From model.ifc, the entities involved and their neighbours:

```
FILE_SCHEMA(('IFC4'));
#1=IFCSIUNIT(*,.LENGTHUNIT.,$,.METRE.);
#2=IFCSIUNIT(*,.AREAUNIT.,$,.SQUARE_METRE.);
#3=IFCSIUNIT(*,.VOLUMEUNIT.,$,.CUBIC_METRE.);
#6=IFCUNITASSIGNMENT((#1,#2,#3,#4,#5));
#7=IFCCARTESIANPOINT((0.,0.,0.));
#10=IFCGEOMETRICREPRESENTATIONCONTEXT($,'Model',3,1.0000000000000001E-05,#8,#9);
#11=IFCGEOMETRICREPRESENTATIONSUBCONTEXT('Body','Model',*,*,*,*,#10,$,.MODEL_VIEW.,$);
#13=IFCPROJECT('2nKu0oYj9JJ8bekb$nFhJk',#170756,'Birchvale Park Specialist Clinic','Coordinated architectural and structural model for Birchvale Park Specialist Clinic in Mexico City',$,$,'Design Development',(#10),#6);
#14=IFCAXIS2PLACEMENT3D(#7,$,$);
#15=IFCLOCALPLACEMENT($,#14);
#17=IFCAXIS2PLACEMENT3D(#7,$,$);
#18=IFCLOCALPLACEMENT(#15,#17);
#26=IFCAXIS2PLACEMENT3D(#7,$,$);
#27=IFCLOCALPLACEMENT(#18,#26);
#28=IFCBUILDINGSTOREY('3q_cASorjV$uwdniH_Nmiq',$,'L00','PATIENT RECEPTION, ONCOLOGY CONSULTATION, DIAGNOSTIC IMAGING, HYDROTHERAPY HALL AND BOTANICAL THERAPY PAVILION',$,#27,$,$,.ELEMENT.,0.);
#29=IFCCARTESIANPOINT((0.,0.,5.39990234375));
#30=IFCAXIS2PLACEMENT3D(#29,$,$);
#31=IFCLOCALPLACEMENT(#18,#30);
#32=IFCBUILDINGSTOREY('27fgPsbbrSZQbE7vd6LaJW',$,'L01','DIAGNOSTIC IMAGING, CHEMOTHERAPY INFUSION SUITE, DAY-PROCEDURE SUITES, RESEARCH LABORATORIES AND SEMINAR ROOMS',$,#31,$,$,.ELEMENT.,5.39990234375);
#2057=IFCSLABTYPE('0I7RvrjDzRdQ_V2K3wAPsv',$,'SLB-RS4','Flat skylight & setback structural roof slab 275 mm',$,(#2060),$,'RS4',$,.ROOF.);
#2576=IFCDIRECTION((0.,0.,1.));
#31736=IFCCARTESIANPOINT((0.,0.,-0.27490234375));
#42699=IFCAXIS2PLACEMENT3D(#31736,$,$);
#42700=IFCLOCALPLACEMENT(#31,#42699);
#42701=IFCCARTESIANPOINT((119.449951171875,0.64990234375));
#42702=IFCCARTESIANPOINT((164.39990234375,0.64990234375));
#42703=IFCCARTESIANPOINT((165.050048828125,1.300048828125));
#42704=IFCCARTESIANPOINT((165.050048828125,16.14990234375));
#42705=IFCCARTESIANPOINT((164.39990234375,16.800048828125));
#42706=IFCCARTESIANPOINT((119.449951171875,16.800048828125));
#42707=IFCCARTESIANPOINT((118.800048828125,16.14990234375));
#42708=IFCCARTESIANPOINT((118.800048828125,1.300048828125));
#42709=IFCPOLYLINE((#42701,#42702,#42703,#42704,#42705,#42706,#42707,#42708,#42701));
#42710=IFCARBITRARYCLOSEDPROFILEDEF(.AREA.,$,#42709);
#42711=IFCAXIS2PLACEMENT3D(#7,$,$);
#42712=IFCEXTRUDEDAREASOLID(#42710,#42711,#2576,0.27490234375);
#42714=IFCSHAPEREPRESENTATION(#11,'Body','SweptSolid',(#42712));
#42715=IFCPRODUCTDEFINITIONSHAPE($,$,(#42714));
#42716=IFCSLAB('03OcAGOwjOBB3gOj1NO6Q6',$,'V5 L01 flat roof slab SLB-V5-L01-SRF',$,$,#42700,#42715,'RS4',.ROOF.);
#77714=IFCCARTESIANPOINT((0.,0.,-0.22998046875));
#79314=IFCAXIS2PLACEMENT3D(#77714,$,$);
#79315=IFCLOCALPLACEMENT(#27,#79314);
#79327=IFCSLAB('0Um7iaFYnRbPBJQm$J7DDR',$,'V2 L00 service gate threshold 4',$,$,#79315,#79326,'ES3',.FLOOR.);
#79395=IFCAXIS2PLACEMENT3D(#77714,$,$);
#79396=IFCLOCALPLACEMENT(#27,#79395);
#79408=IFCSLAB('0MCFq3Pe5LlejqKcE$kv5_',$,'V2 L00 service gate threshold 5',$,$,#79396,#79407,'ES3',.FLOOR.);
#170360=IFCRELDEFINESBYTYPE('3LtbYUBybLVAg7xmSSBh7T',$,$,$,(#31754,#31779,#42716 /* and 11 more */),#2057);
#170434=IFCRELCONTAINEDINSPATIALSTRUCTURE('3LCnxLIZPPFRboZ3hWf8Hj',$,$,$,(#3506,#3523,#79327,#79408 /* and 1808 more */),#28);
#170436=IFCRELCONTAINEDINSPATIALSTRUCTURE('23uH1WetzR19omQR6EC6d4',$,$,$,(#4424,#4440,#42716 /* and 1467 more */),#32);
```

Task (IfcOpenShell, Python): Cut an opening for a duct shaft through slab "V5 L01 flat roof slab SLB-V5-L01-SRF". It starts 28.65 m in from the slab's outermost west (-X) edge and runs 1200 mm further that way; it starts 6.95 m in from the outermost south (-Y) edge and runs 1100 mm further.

```python
import numpy as np
import ifcopenshell
import ifcopenshell.api.feature
import ifcopenshell.api.geometry
import ifcopenshell.api.root
import ifcopenshell.geom
import ifcopenshell.util.placement
import ifcopenshell.util.representation
import ifcopenshell.util.shape
import ifcopenshell.util.unit

model = ifcopenshell.open("model.ifc")
unit_scale = ifcopenshell.util.unit.calculate_unit_scale(model)
settings = ifcopenshell.geom.settings()


def volume(element):
    """Net volume in cubic metres, openings subtracted."""
    shape = ifcopenshell.geom.create_shape(settings, element)
    return ifcopenshell.util.shape.get_volume(shape.geometry)


slab = model.by_guid("03OcAGOwjOBB3gOj1NO6Q6")
before = volume(slab)

# Extent in the slab's own axes, in metres. The edges named are its -X and -Y sides.
slab_shape = ifcopenshell.geom.create_shape(settings, slab)
vertices = ifcopenshell.util.shape.get_vertices(slab_shape.geometry)
x_min, y_min, bottom = vertices.min(axis=0)
top = vertices[:, 2].max()

opening = ifcopenshell.api.root.create_entity(model, ifc_class="IfcOpeningElement", name="Duct shaft opening", predefined_type="OPENING")
context = ifcopenshell.util.representation.get_context(model, "Model", "Body", "MODEL_VIEW")
width, depth = 1.2, 1.1
outline = [(0.0, 0.0), (width, 0.0), (width, depth), (0.0, depth), (0.0, 0.0)]
# Overshoot both faces by 50 mm so the cut is clean.
shape = ifcopenshell.api.geometry.add_slab_representation(
    model, context=context, depth=top - bottom + 0.1, polyline=outline
)
ifcopenshell.api.geometry.assign_representation(model, product=opening, representation=shape)

matrix = ifcopenshell.util.placement.get_local_placement(slab.ObjectPlacement)
matrix[:, 3] = matrix @ np.append(np.array([x_min + 28.65, y_min + 6.95, bottom - 0.05]) / unit_scale, 1.0)
ifcopenshell.api.geometry.edit_object_placement(model, product=opening, matrix=matrix, is_si=False)
ifcopenshell.api.feature.add_feature(model, feature=opening, element=slab)

after = volume(slab)

print(f"slab volume {before:.3f} -> {after:.3f} m3")

model.write("model_rev.ifc")
```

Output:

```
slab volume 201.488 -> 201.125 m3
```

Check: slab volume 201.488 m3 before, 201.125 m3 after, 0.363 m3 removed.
